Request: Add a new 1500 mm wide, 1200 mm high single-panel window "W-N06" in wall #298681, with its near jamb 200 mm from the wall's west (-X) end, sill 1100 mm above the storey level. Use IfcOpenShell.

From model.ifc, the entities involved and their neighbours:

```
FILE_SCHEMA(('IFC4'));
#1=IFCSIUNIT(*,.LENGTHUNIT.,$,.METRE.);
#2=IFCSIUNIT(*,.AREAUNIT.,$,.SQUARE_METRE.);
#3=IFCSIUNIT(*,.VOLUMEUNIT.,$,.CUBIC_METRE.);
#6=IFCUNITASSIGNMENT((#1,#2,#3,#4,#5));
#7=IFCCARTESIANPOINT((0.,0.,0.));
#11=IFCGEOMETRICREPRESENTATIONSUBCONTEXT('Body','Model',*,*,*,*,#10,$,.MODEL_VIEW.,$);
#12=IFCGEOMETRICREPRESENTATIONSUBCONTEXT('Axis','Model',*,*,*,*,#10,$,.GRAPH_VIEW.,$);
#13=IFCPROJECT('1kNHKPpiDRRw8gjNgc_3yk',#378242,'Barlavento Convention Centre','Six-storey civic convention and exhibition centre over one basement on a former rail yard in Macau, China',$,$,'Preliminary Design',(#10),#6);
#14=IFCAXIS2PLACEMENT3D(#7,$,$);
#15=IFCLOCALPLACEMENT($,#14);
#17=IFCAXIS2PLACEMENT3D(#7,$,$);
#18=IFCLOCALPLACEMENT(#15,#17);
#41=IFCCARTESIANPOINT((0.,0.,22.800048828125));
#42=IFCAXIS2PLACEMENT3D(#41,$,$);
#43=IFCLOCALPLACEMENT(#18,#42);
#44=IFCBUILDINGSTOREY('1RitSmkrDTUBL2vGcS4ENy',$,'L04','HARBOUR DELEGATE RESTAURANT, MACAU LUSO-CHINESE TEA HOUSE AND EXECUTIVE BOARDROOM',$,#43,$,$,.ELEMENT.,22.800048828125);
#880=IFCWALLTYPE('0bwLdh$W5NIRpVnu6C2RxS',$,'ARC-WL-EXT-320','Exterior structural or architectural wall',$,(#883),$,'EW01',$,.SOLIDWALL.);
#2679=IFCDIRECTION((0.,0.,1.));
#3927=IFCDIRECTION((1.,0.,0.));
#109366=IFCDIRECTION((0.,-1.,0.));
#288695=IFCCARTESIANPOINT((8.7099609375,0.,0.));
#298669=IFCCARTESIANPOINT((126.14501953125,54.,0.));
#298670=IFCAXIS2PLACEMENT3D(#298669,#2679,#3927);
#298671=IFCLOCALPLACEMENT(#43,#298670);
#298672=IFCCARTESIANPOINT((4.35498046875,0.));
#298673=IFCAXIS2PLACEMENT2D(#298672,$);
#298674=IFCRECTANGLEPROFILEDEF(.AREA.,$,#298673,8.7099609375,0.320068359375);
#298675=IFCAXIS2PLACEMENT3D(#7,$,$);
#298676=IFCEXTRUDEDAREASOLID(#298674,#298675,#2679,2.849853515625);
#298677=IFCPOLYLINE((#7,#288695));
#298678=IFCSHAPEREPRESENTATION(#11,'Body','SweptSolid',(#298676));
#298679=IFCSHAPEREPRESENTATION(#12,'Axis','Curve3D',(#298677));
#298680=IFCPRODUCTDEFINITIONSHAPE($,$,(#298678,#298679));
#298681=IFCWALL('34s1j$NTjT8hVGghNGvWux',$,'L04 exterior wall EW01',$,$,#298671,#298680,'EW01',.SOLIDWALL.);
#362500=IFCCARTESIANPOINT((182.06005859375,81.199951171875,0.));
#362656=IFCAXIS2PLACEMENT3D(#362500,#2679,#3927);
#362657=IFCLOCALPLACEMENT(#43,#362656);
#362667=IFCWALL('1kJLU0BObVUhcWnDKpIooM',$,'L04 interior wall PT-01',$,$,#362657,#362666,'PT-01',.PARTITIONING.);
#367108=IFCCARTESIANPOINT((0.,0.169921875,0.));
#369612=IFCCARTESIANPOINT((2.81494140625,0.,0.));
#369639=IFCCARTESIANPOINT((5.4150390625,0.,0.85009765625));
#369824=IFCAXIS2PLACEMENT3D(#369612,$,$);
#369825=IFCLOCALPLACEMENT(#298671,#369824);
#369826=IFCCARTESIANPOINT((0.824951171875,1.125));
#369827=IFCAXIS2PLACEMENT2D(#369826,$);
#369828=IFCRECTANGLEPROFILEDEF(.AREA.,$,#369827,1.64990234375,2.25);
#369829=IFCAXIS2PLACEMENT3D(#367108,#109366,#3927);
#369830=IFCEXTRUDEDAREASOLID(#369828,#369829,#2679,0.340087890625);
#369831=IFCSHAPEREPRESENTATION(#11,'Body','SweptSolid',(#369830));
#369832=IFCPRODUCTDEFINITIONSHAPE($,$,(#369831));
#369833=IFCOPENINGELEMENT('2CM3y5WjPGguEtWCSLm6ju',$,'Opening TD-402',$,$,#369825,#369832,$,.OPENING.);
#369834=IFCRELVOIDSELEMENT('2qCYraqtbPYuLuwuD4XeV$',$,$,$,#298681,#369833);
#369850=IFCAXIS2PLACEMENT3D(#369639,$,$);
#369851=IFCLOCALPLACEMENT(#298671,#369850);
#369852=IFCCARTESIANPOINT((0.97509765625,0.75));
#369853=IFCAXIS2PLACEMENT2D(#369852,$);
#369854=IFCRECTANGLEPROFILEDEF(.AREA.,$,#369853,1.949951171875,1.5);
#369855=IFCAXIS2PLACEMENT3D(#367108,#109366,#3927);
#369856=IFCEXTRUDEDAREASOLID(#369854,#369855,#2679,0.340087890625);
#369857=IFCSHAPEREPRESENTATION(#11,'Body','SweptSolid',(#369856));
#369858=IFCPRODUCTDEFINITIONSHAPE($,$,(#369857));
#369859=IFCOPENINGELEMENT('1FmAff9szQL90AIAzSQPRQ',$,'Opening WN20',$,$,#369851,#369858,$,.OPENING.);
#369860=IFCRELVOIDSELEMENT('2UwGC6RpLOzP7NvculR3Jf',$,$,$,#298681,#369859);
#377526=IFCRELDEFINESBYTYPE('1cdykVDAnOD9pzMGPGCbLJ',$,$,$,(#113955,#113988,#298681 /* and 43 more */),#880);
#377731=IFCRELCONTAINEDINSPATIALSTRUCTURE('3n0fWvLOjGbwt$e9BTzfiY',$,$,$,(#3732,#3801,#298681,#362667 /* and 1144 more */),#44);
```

```python
import numpy as np
import ifcopenshell
import ifcopenshell.api.feature
import ifcopenshell.api.geometry
import ifcopenshell.api.root
import ifcopenshell.api.spatial
import ifcopenshell.geom
import ifcopenshell.util.element
import ifcopenshell.util.placement
import ifcopenshell.util.representation
import ifcopenshell.util.shape
import ifcopenshell.util.unit

model = ifcopenshell.open("model.ifc")
unit_scale = ifcopenshell.util.unit.calculate_unit_scale(model)
settings = ifcopenshell.geom.settings()


def volume(element):
    """Net volume in cubic metres, openings subtracted."""
    shape = ifcopenshell.geom.create_shape(settings, element)
    return ifcopenshell.util.shape.get_volume(shape.geometry)


wall = model.by_guid("34s1j$NTjT8hVGghNGvWux")
storey = ifcopenshell.util.element.get_container(wall, ifc_class="IfcBuildingStorey")
context = ifcopenshell.util.representation.get_context(model, "Model", "Body", "MODEL_VIEW")
before = volume(wall)

width, height, from_end, sill = 1.5, 1.2, 0.2, 1.1  # metres

# The wall runs along its own X axis, and the end named is its -X end.
wall_shape = ifcopenshell.geom.create_shape(settings, wall)
x, y, z = ifcopenshell.util.shape.get_vertices(wall_shape.geometry).T
start = x.min() + from_end
face, thickness = float(y.min()), float(y.max() - y.min())
wall_matrix = ifcopenshell.util.placement.get_local_placement(wall.ObjectPlacement)
level = ifcopenshell.util.placement.get_local_placement(storey.ObjectPlacement)[2, 3]


def in_wall(x, y):
    """Placement at x, y metres in the wall's axes, at sill height."""
    matrix = wall_matrix.copy()
    matrix[:, 3] = wall_matrix @ np.array([x / unit_scale, y / unit_scale, 0.0, 1.0])
    matrix[2, 3] = level + sill / unit_scale
    return matrix


# Opening: a box that overshoots both wall faces by 50 mm.
opening = ifcopenshell.api.root.create_entity(model, ifc_class="IfcOpeningElement", predefined_type="OPENING")
box = ifcopenshell.api.geometry.add_wall_representation(
    model, context=context, length=width, height=height, thickness=thickness + 0.1
)
ifcopenshell.api.geometry.assign_representation(model, product=opening, representation=box)
ifcopenshell.api.geometry.edit_object_placement(model, product=opening, matrix=in_wall(start, face - 0.05), is_si=False)
ifcopenshell.api.feature.add_feature(model, feature=opening, element=wall)

window = ifcopenshell.api.root.create_entity(model, ifc_class="IfcWindow", name="W-N06", predefined_type="WINDOW")
window.OverallWidth, window.OverallHeight = width / unit_scale, height / unit_scale
window.PartitioningType = "SINGLE_PANEL"
body = ifcopenshell.api.geometry.add_window_representation(
    model,
    context=context,
    overall_width=window.OverallWidth,
    overall_height=window.OverallHeight,
    partition_type="SINGLE_PANEL",
)
ifcopenshell.api.geometry.assign_representation(model, product=window, representation=body)
ifcopenshell.api.spatial.assign_container(model, products=[window], relating_structure=storey)
ifcopenshell.api.feature.add_filling(model, opening=opening, element=window)

# Centre the window in the wall's thickness.
ifcopenshell.api.geometry.edit_object_placement(model, product=window, matrix=in_wall(start, face), is_si=False)
window_shape = ifcopenshell.geom.create_shape(settings, window)
depth = ifcopenshell.util.shape.get_vertices(window_shape.geometry)[:, 1]
offset = face + thickness / 2 - (depth.min() + depth.max()) / 2
ifcopenshell.api.geometry.edit_object_placement(model, product=window, matrix=in_wall(start, offset), is_si=False)

after = volume(wall)

print(f"wall volume {before:.3f} -> {after:.3f} m3")

model.write("model-out.ifc")
```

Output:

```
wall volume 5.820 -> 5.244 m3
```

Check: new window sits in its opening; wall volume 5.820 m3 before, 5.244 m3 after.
